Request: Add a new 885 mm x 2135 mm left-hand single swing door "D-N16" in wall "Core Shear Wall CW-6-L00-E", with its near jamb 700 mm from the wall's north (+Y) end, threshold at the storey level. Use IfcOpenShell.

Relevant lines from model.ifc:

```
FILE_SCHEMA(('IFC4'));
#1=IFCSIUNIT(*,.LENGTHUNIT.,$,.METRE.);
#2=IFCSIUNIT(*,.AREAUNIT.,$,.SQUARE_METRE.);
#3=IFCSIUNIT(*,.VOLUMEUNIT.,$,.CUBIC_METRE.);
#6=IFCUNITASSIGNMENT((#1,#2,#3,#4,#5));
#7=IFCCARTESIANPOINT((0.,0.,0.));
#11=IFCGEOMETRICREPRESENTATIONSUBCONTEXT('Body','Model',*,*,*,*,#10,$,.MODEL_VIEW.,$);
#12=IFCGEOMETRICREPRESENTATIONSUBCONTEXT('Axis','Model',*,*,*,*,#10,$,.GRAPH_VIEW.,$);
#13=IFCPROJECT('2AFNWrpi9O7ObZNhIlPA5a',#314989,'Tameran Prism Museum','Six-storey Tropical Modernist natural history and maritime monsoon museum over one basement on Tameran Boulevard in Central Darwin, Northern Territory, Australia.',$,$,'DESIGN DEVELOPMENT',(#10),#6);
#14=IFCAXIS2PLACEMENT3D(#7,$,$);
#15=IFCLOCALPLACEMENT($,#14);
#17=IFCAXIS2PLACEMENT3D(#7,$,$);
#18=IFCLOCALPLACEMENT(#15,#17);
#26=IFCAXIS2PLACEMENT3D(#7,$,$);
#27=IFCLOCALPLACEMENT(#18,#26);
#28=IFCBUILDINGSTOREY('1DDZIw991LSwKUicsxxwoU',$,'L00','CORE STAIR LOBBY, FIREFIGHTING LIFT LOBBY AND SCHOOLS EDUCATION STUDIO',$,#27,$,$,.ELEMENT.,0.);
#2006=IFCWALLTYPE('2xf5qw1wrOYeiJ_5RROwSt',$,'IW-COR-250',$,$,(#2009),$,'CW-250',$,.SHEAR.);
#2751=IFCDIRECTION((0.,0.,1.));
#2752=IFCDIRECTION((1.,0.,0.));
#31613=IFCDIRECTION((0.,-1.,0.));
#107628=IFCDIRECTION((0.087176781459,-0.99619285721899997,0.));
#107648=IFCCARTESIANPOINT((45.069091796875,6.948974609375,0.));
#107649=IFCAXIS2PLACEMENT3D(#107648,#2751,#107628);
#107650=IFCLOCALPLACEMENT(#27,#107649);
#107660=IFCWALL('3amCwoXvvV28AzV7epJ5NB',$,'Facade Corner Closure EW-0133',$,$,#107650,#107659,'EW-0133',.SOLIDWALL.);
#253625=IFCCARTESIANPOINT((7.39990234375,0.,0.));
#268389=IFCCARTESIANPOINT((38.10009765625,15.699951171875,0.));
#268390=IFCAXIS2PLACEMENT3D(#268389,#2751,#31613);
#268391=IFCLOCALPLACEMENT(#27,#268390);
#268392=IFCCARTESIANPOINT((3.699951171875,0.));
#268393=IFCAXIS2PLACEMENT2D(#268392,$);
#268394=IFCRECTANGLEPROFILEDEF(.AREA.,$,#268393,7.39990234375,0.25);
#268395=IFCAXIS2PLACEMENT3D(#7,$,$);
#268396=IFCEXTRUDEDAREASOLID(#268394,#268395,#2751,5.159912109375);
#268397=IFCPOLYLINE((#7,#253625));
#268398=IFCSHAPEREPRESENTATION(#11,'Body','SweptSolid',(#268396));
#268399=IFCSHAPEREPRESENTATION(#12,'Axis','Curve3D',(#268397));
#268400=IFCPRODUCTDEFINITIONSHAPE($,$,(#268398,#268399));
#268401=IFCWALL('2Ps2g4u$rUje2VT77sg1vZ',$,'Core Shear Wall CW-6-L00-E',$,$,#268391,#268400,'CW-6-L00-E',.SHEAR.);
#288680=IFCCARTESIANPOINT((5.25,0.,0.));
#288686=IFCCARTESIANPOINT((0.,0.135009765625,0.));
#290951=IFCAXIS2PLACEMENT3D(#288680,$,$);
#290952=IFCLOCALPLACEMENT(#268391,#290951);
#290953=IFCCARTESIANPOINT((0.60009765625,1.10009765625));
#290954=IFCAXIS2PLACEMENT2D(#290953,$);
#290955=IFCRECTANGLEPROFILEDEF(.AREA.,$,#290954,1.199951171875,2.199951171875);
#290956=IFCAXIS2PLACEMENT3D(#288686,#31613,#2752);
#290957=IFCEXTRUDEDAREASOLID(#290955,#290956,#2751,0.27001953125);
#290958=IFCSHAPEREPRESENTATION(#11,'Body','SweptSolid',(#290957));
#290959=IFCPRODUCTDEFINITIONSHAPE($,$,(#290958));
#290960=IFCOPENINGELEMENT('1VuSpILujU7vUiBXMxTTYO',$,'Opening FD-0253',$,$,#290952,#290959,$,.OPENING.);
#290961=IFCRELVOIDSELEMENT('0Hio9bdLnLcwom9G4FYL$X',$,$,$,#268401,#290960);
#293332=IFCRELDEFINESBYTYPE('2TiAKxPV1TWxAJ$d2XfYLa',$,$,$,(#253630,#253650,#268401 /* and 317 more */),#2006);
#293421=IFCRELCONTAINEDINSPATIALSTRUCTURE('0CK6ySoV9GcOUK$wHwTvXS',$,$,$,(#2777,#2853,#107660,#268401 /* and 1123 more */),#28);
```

```python
import numpy as np
import ifcopenshell
import ifcopenshell.api.feature
import ifcopenshell.api.geometry
import ifcopenshell.api.root
import ifcopenshell.api.spatial
import ifcopenshell.geom
import ifcopenshell.util.element
import ifcopenshell.util.placement
import ifcopenshell.util.representation
import ifcopenshell.util.shape
import ifcopenshell.util.unit

model = ifcopenshell.open("model.ifc")
unit_scale = ifcopenshell.util.unit.calculate_unit_scale(model)
settings = ifcopenshell.geom.settings()


def volume(element):
    """Net volume in cubic metres, openings subtracted."""
    shape = ifcopenshell.geom.create_shape(settings, element)
    return ifcopenshell.util.shape.get_volume(shape.geometry)


wall = model.by_guid("2Ps2g4u$rUje2VT77sg1vZ")
storey = ifcopenshell.util.element.get_container(wall, ifc_class="IfcBuildingStorey")
context = ifcopenshell.util.representation.get_context(model, "Model", "Body", "MODEL_VIEW")
before = volume(wall)

width, height, from_end, sill = 0.885, 2.135, 0.7, 0.0  # metres

# The wall runs along its own X axis, and the end named is its -X end.
wall_shape = ifcopenshell.geom.create_shape(settings, wall)
x, y, z = ifcopenshell.util.shape.get_vertices(wall_shape.geometry).T
start = x.min() + from_end
face, thickness = float(y.min()), float(y.max() - y.min())
wall_matrix = ifcopenshell.util.placement.get_local_placement(wall.ObjectPlacement)
level = ifcopenshell.util.placement.get_local_placement(storey.ObjectPlacement)[2, 3]


def in_wall(x, y):
    """Placement at x, y metres in the wall's axes, at sill height."""
    matrix = wall_matrix.copy()
    matrix[:, 3] = wall_matrix @ np.array([x / unit_scale, y / unit_scale, 0.0, 1.0])
    matrix[2, 3] = level + sill / unit_scale
    return matrix


# Opening: a box that overshoots both wall faces by 50 mm.
opening = ifcopenshell.api.root.create_entity(model, ifc_class="IfcOpeningElement", predefined_type="OPENING")
box = ifcopenshell.api.geometry.add_wall_representation(
    model, context=context, length=width, height=height, thickness=thickness + 0.1
)
ifcopenshell.api.geometry.assign_representation(model, product=opening, representation=box)
ifcopenshell.api.geometry.edit_object_placement(model, product=opening, matrix=in_wall(start, face - 0.05), is_si=False)
ifcopenshell.api.feature.add_feature(model, feature=opening, element=wall)

door = ifcopenshell.api.root.create_entity(model, ifc_class="IfcDoor", name="D-N16", predefined_type="DOOR")
door.OverallWidth, door.OverallHeight = width / unit_scale, height / unit_scale
door.OperationType = "SINGLE_SWING_LEFT"
body = ifcopenshell.api.geometry.add_door_representation(
    model,
    context=context,
    overall_width=door.OverallWidth,
    overall_height=door.OverallHeight,
    operation_type="SINGLE_SWING_LEFT",
    lining_properties={"LiningDepth": thickness / unit_scale, "ThresholdDepth": thickness / unit_scale},
)
ifcopenshell.api.geometry.assign_representation(model, product=door, representation=body)
ifcopenshell.api.spatial.assign_container(model, products=[door], relating_structure=storey)
ifcopenshell.api.feature.add_filling(model, opening=opening, element=door)

# The lining spans the wall, so the door starts at the wall face.
ifcopenshell.api.geometry.edit_object_placement(model, product=door, matrix=in_wall(start, face), is_si=False)

after = volume(wall)

print(f"wall volume {before:.3f} -> {after:.3f} m3")

model.write("model_edited.ifc")
```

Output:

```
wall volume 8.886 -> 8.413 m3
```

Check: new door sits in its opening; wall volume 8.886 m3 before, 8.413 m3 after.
